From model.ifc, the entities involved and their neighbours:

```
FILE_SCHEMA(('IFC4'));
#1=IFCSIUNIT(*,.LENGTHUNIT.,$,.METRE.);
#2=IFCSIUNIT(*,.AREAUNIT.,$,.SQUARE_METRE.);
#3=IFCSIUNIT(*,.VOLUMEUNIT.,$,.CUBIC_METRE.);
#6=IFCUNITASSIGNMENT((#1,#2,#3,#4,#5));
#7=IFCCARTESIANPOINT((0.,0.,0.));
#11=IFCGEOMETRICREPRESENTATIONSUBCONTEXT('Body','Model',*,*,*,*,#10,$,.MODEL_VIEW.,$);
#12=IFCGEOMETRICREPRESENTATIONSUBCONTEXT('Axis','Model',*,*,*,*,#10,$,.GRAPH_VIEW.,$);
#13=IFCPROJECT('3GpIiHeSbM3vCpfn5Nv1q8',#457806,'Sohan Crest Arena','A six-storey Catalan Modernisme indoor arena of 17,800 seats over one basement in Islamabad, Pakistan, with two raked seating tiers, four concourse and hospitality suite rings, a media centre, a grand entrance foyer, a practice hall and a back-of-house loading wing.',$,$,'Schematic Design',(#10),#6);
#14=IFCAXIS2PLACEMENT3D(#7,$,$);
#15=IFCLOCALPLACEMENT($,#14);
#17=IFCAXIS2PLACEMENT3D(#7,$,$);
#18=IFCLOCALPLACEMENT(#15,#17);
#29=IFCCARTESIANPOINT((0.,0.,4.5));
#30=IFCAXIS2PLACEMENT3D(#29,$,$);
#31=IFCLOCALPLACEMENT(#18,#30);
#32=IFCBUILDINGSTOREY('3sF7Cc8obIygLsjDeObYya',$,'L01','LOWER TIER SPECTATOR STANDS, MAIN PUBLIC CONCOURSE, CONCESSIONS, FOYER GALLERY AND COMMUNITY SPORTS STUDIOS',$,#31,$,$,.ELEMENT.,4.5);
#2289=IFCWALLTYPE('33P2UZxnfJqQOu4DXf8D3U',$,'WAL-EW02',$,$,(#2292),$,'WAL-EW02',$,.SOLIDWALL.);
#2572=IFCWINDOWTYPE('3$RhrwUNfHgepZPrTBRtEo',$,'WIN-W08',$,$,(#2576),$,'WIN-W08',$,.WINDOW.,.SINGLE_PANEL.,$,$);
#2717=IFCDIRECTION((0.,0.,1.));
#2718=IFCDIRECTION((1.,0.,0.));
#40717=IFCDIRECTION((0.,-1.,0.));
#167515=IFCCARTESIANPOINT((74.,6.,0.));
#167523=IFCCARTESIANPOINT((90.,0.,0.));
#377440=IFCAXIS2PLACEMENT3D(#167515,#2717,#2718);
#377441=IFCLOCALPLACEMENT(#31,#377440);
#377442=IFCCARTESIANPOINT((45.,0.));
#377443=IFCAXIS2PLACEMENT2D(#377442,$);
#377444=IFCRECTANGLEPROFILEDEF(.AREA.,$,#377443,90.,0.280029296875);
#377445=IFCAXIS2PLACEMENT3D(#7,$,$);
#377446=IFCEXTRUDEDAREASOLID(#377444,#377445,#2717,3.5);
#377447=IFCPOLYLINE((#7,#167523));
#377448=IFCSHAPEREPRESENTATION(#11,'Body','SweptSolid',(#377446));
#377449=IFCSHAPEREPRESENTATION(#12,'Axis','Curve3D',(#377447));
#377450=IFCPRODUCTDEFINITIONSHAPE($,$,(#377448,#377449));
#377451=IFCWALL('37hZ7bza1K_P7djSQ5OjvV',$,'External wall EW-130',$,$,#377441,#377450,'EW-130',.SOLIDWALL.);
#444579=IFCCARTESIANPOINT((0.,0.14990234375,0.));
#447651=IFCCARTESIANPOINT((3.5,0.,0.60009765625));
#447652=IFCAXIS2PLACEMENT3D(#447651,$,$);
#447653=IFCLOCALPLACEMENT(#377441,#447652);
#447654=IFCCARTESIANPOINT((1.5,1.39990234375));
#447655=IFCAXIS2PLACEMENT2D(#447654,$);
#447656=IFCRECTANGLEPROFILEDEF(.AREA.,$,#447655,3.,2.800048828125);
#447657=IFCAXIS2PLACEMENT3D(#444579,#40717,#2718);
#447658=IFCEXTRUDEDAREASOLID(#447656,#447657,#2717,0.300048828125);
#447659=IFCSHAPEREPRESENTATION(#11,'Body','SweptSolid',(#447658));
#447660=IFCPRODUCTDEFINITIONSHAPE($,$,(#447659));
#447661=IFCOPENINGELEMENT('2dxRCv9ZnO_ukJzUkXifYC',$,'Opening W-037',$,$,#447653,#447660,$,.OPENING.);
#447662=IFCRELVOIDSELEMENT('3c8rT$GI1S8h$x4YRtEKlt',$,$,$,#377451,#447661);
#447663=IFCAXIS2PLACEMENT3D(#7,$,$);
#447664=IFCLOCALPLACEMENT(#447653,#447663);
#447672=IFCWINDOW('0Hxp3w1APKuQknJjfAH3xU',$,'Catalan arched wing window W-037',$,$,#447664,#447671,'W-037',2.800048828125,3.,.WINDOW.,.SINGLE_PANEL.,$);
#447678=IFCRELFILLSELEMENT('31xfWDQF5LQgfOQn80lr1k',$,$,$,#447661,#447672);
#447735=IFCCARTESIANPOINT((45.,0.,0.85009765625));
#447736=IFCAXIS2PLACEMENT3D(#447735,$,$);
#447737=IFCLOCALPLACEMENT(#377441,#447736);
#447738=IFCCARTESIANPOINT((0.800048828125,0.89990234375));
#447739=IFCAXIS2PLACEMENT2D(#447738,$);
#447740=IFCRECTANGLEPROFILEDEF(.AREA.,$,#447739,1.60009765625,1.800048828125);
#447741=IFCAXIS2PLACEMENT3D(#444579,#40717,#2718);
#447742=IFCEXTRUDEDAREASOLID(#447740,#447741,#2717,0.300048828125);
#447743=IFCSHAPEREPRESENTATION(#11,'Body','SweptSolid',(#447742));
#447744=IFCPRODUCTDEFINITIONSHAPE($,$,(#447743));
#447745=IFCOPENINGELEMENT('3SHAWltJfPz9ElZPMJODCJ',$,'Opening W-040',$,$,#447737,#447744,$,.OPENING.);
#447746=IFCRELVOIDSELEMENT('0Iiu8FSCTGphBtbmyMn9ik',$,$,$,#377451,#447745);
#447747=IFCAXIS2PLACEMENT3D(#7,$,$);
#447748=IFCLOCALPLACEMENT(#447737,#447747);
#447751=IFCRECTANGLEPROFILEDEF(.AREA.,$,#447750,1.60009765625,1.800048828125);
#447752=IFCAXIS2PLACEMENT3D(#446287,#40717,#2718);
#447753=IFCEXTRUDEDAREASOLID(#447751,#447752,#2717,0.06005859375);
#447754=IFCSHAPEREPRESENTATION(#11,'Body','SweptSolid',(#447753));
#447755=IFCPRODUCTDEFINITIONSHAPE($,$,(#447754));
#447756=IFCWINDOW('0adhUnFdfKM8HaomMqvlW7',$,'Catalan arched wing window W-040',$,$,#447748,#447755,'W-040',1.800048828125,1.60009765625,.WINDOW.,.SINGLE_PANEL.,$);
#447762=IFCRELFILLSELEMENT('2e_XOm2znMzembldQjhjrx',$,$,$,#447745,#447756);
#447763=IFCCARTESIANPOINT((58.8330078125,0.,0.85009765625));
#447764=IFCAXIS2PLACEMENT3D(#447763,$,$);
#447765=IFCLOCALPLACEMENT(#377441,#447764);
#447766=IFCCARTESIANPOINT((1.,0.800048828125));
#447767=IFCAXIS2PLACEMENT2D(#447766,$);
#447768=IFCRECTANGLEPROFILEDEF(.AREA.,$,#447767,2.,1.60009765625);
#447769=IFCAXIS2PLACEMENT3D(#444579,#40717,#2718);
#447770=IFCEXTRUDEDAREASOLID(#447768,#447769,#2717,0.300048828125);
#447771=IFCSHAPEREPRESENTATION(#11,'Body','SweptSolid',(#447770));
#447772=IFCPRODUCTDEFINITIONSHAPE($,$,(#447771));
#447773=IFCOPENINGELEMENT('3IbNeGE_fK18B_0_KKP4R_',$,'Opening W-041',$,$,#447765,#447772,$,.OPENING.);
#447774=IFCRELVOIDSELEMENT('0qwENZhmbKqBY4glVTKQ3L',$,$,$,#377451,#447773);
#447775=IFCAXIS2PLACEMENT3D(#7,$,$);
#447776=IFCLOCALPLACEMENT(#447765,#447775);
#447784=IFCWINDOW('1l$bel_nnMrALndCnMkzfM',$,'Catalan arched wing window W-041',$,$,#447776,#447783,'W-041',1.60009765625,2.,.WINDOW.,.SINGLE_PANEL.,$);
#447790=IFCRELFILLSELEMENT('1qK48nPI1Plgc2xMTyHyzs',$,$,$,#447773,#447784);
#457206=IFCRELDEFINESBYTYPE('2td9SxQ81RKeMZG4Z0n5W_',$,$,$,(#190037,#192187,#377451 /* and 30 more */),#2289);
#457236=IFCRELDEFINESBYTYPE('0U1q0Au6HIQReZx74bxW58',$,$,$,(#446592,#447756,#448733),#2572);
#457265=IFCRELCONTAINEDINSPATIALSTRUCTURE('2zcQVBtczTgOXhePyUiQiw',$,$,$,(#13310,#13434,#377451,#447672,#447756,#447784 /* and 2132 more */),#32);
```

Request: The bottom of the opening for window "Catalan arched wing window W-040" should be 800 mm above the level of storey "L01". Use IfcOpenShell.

```python
import numpy as np
import ifcopenshell
import ifcopenshell.api.geometry
import ifcopenshell.geom
import ifcopenshell.util.element
import ifcopenshell.util.placement
import ifcopenshell.util.shape
import ifcopenshell.util.unit

model = ifcopenshell.open("model.ifc")
unit_scale = ifcopenshell.util.unit.calculate_unit_scale(model)

window = model.by_id(447756)
opening = window.FillsVoids[0].RelatingOpeningElement
storey = ifcopenshell.util.element.get_container(window, ifc_class="IfcBuildingStorey")
level = ifcopenshell.util.placement.get_local_placement(storey.ObjectPlacement)[2, 3]

# The opening's origin need not be at the sill, so measure its lowest point.
shape = ifcopenshell.geom.create_shape(ifcopenshell.geom.settings(), opening)
bottom = ifcopenshell.util.shape.get_shape_bottom_elevation(shape, shape.geometry) / unit_scale
dz = level + 0.8 / unit_scale - bottom

shift = np.array([0.0, 0.0, dz])
# The window is placed relative to its opening, so it follows when the opening moves.
matrix = ifcopenshell.util.placement.get_local_placement(opening.ObjectPlacement)
matrix[:3, 3] += shift
ifcopenshell.api.geometry.edit_object_placement(
    model, product=opening, matrix=matrix, is_si=False, should_transform_children=True
)

print(f"moved by {dz * unit_scale:+.3f} m")

model.write("model_v2.ifc")
```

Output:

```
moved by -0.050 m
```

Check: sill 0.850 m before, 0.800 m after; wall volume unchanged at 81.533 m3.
